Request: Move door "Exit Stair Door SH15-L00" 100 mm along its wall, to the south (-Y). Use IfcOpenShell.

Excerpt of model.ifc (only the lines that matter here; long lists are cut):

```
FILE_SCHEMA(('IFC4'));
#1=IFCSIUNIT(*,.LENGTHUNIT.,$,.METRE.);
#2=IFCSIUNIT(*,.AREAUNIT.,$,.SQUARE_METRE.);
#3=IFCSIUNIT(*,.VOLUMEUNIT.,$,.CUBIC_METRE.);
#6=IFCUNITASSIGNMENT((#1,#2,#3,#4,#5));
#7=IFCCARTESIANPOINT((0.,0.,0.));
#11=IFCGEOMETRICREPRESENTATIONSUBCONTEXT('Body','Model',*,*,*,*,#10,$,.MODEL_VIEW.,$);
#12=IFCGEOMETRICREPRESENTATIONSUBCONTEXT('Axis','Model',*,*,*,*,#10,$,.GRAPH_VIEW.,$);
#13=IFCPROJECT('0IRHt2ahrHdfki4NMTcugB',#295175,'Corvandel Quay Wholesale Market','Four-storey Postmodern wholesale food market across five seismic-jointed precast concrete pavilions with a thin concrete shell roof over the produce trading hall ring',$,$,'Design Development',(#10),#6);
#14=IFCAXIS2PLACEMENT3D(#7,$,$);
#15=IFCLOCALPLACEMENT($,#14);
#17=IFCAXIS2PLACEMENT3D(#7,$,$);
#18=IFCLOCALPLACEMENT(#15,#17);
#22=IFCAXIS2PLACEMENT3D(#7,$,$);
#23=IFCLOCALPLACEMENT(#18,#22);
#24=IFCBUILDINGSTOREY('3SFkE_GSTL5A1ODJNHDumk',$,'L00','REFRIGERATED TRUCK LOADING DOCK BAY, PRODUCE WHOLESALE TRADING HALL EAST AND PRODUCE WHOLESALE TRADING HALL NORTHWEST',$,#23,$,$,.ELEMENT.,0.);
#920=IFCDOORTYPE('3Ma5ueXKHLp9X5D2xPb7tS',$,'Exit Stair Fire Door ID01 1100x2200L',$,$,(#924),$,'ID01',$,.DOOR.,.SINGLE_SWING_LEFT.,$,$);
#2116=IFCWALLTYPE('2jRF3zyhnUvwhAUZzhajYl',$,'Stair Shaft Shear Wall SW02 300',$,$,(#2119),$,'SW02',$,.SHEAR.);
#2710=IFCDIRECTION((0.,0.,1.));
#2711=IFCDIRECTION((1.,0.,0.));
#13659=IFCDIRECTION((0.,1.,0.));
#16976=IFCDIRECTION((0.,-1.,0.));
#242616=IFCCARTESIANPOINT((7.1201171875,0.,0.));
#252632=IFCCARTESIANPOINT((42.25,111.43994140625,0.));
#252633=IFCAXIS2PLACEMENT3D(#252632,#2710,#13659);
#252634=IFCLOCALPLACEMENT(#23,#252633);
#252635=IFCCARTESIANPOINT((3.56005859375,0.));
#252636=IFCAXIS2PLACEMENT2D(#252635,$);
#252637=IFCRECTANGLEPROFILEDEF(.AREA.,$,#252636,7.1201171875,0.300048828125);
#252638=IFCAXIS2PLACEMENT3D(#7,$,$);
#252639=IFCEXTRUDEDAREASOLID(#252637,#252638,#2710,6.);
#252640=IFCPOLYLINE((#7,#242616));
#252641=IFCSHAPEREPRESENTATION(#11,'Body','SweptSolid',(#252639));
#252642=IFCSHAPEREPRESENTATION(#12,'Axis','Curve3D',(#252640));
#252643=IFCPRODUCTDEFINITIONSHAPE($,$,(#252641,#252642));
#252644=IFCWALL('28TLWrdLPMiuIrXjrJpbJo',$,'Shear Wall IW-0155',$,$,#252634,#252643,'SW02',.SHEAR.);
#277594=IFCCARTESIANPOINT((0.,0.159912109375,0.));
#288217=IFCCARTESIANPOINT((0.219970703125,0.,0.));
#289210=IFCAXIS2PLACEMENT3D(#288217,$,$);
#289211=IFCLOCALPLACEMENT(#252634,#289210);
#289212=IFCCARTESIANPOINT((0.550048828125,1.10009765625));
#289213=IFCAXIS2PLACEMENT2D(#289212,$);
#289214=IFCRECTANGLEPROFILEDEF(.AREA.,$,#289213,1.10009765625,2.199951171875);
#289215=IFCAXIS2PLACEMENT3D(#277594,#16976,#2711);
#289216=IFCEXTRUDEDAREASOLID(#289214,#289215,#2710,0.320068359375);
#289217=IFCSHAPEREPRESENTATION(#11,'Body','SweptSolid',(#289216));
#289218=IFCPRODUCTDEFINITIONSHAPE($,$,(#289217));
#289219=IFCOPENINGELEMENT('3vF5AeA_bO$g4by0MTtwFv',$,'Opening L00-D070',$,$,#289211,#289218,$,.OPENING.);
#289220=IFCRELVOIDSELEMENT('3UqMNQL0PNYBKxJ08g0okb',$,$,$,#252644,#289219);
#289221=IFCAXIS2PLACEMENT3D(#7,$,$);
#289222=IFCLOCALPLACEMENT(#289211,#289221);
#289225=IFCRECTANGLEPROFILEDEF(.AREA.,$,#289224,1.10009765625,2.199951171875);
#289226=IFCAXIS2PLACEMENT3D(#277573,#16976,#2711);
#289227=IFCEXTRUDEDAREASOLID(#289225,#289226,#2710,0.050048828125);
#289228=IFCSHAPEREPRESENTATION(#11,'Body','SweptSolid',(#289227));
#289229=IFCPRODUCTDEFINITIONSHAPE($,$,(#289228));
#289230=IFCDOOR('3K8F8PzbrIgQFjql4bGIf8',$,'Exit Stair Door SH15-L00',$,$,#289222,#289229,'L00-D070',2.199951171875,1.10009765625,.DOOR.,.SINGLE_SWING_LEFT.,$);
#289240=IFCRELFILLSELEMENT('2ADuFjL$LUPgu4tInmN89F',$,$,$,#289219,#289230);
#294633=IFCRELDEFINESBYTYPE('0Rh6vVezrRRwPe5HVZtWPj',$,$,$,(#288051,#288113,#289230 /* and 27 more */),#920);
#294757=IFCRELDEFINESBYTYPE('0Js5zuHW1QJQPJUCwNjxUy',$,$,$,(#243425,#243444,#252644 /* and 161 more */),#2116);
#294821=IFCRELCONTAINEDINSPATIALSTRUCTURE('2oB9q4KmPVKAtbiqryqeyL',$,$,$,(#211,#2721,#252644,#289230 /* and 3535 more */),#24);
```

```python
import ifcopenshell
import ifcopenshell.api.geometry
import ifcopenshell.util.placement

model = ifcopenshell.open("model.ifc")

door = model.by_id(289230)
opening = door.FillsVoids[0].RelatingOpeningElement
wall = opening.VoidsElements[0].RelatingBuildingElement

wall_matrix = ifcopenshell.util.placement.get_local_placement(wall.ObjectPlacement)
shift = wall_matrix[:3, 0] * -0.1
before = ifcopenshell.util.placement.get_local_placement(door.ObjectPlacement)[:3, 3].copy()

# The door is placed relative to its opening, so it follows when the opening moves.
matrix = ifcopenshell.util.placement.get_local_placement(opening.ObjectPlacement)
matrix[:3, 3] += shift
ifcopenshell.api.geometry.edit_object_placement(
    model, product=opening, matrix=matrix, is_si=False, should_transform_children=True
)

after = ifcopenshell.util.placement.get_local_placement(door.ObjectPlacement)[:3, 3]
print("door moved by", (after - before).round(3) + 0.0)

model.write("model_updated.ifc")
```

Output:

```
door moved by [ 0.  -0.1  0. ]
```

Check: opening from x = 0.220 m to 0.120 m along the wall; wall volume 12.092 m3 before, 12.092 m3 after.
